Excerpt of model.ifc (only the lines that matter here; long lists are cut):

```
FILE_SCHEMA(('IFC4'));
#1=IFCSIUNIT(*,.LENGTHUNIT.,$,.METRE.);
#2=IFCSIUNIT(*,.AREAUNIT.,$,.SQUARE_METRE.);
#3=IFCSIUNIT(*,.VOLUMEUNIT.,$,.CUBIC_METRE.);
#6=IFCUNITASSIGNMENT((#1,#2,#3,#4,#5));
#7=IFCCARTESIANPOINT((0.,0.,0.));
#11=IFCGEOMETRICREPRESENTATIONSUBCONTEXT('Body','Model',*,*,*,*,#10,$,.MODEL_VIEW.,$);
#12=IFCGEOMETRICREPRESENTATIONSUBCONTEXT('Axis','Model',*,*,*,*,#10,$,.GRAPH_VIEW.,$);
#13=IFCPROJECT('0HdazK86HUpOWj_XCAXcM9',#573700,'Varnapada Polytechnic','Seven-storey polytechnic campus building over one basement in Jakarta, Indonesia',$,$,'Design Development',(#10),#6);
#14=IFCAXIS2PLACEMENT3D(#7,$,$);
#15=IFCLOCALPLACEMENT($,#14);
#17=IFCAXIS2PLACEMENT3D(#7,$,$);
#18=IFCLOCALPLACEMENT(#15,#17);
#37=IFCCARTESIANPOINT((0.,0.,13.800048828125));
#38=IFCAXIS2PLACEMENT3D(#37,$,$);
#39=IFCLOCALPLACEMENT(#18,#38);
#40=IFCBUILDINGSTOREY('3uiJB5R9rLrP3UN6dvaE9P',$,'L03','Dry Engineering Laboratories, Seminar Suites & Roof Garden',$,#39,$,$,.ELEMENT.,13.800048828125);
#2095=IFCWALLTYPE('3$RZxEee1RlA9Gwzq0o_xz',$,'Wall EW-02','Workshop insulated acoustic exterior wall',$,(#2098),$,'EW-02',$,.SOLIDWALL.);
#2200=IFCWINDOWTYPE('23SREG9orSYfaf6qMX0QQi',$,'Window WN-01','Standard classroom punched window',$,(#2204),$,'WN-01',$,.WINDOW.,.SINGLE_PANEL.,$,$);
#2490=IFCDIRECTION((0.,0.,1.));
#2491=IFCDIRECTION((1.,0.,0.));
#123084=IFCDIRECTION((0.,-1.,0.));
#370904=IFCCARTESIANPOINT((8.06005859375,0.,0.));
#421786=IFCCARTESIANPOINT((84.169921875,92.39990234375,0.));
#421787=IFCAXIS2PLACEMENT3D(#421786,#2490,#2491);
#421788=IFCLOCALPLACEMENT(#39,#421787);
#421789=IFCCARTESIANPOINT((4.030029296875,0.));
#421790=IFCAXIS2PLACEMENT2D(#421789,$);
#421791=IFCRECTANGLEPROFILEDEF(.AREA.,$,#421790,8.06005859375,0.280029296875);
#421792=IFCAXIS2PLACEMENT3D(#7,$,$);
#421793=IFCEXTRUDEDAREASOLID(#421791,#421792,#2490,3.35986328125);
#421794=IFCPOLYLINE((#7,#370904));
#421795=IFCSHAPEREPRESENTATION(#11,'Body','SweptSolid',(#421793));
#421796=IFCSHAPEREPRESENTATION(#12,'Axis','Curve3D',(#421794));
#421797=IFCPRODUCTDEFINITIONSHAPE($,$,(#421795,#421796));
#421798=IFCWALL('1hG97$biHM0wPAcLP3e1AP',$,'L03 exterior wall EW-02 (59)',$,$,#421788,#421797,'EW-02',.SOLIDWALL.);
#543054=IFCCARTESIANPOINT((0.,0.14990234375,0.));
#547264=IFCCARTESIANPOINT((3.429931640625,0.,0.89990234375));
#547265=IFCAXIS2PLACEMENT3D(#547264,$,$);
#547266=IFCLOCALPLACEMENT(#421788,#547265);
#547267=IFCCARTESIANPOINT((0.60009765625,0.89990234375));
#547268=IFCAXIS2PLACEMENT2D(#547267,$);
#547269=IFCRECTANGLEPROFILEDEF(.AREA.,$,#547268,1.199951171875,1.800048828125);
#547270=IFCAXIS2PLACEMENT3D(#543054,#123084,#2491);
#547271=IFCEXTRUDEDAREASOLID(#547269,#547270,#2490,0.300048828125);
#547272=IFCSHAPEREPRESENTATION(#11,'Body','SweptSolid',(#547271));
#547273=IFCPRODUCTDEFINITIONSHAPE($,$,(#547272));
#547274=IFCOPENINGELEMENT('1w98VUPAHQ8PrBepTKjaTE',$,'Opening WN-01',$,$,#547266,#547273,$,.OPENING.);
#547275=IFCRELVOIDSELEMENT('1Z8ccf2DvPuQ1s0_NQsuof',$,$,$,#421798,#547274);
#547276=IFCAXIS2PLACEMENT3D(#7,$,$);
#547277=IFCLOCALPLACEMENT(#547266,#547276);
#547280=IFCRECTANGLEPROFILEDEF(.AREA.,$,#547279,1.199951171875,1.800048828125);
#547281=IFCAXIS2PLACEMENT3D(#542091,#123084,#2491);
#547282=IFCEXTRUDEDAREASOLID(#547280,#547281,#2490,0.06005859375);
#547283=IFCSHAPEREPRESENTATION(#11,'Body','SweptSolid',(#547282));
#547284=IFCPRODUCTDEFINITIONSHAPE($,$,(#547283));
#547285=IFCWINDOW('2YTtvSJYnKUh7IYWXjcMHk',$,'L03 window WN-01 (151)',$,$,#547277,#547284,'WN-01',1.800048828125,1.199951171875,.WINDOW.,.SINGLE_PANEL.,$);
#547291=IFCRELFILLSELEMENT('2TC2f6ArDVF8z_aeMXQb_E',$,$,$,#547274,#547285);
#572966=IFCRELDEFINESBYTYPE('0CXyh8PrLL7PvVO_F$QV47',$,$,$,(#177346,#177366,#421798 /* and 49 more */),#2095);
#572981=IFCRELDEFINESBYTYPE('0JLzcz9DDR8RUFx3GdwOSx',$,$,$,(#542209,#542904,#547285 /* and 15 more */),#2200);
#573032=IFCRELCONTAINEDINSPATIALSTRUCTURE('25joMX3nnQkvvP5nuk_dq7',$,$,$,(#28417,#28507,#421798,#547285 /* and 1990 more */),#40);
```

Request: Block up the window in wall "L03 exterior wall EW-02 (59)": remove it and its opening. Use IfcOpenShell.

```python
import ifcopenshell
import ifcopenshell.api.feature
import ifcopenshell.api.root
import ifcopenshell.geom
import ifcopenshell.util.shape

model = ifcopenshell.open("model.ifc")
settings = ifcopenshell.geom.settings()


def volume(element):
    """Net volume in cubic metres, openings subtracted."""
    shape = ifcopenshell.geom.create_shape(settings, element)
    return ifcopenshell.util.shape.get_volume(shape.geometry)


window = model.by_id(547285)
opening = window.FillsVoids[0].RelatingOpeningElement
wall = opening.VoidsElements[0].RelatingBuildingElement
before = volume(wall)

ifcopenshell.api.root.remove_product(model, product=window)
ifcopenshell.api.feature.remove_feature(model, feature=opening)

after = volume(wall)

print(f"wall volume {before:.3f} -> {after:.3f} m3")

model.write("model-out.ifc")
```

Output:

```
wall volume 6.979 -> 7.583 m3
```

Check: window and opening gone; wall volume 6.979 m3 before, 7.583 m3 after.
